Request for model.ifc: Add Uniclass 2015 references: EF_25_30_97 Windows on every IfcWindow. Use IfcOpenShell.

First a look at what the model holds.

```python
import ifcopenshell

model = ifcopenshell.open("model.ifc")
print(model.schema)
print("classifications:", [c.Name for c in model.by_type("IfcClassification")])
for ifc_class in ("IfcDoor", "IfcRoof", "IfcStair", "IfcWall", "IfcWindow"):
    print(ifc_class, len(model.by_type(ifc_class)))
```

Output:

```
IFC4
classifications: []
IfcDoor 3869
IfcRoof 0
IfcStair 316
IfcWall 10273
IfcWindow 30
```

```python
import ifcopenshell
import ifcopenshell.api.classification

model = ifcopenshell.open("model.ifc")

system = ifcopenshell.api.classification.add_classification(model, classification="Uniclass 2015")

codes = {
    "IfcWindow": ("EF_25_30_97", "Windows"),
}
for ifc_class, (code, name) in codes.items():
    products = model.by_type(ifc_class)
    ifcopenshell.api.classification.add_reference(
        model, products=products, classification=system, identification=code, name=name
    )
    print(code, len(products))

model.write("model_updated.ifc")
```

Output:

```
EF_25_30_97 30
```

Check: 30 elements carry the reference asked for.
